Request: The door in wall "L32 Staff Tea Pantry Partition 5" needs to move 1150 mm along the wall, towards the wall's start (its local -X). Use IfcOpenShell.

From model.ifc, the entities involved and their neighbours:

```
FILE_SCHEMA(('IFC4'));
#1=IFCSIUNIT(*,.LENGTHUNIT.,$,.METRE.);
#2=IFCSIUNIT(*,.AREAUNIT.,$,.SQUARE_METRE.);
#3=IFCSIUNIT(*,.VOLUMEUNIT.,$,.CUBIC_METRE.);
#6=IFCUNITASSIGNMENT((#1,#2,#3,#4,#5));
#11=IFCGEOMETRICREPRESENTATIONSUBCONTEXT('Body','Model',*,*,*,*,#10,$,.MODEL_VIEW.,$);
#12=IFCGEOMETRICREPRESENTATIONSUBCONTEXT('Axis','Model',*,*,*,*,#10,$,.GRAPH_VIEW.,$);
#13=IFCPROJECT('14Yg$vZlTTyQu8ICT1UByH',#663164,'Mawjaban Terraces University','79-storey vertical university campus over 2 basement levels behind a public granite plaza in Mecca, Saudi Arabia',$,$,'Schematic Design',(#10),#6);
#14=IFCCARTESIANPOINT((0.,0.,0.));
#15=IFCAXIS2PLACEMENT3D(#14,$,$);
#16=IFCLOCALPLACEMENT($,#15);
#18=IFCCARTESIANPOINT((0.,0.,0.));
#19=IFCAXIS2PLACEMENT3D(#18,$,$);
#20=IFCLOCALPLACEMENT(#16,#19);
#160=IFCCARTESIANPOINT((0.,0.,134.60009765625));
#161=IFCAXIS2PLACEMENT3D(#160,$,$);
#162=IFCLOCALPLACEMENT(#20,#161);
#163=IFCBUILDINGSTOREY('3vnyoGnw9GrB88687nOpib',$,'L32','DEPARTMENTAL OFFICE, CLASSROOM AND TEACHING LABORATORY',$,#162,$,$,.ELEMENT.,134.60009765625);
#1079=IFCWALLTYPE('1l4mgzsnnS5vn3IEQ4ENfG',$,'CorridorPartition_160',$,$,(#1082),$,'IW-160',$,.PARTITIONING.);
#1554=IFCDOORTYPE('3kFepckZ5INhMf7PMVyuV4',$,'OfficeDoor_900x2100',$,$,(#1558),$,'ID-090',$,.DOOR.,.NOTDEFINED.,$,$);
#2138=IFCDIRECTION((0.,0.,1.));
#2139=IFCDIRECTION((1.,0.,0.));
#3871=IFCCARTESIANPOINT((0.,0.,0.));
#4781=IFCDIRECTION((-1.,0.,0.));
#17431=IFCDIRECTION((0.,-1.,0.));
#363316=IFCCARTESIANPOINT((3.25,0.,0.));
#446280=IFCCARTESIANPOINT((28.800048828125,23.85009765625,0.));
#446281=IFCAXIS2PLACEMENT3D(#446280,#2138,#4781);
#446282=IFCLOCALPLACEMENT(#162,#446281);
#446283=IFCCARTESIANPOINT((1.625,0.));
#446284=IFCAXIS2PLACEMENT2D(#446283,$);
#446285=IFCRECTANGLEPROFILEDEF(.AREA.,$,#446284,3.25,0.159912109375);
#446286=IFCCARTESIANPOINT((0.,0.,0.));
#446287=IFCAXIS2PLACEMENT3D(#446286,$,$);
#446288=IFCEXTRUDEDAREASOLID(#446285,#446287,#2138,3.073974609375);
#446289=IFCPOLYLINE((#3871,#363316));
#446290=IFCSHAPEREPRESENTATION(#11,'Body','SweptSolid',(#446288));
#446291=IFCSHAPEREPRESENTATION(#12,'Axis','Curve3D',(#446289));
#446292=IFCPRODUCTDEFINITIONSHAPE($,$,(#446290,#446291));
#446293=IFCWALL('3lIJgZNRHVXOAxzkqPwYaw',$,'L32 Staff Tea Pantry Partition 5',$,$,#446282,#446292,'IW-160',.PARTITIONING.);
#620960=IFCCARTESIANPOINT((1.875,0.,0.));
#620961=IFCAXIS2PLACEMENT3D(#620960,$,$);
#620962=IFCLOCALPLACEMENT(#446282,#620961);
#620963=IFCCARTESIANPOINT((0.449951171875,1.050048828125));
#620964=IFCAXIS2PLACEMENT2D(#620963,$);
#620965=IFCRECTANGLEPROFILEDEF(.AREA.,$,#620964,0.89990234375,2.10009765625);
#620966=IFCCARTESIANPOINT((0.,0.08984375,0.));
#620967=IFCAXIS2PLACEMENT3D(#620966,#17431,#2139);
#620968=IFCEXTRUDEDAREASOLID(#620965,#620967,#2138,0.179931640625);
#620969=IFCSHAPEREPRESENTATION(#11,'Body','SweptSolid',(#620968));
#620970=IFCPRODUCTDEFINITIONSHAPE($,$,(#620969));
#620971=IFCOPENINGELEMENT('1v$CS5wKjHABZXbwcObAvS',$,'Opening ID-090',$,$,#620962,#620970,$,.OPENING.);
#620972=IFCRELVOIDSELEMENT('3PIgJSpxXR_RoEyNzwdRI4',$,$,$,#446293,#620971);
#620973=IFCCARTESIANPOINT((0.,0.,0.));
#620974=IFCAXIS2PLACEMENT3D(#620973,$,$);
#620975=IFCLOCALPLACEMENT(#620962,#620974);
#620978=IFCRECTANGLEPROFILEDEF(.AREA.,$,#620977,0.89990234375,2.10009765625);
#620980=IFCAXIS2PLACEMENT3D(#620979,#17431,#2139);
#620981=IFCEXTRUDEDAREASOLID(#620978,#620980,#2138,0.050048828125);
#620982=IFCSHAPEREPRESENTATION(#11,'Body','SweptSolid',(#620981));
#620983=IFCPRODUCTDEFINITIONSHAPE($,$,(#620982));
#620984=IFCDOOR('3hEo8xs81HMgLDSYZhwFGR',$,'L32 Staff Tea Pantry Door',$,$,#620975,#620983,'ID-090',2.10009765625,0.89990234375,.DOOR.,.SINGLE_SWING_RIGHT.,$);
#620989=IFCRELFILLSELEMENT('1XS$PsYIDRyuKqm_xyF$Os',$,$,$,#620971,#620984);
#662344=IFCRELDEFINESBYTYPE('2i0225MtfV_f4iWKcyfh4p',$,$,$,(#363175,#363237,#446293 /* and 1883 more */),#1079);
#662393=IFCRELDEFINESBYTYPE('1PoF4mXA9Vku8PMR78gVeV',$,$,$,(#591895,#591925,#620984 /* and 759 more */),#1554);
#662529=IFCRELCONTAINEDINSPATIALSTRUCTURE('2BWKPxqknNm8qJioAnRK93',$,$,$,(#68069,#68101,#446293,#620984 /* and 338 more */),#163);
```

```python
import ifcopenshell
import ifcopenshell.api.geometry
import ifcopenshell.util.placement

model = ifcopenshell.open("model.ifc")

door = model.by_guid("3hEo8xs81HMgLDSYZhwFGR")
opening = door.FillsVoids[0].RelatingOpeningElement
wall = opening.VoidsElements[0].RelatingBuildingElement

wall_matrix = ifcopenshell.util.placement.get_local_placement(wall.ObjectPlacement)
shift = wall_matrix[:3, 0] * -1.15
before = ifcopenshell.util.placement.get_local_placement(door.ObjectPlacement)[:3, 3].copy()

# The door is placed relative to its opening, so it follows when the opening moves.
matrix = ifcopenshell.util.placement.get_local_placement(opening.ObjectPlacement)
matrix[:3, 3] += shift
ifcopenshell.api.geometry.edit_object_placement(
    model, product=opening, matrix=matrix, is_si=False, should_transform_children=True
)

after = ifcopenshell.util.placement.get_local_placement(door.ObjectPlacement)[:3, 3]
print("door moved by", (after - before).round(3) + 0.0)

model.write("model_edited.ifc")
```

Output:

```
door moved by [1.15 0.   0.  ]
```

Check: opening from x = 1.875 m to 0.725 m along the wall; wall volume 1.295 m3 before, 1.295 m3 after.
